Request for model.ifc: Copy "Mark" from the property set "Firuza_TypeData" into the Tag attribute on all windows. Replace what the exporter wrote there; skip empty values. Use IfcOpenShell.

First a look at what the model holds.

```python
import ifcopenshell
import ifcopenshell.util.element

model = ifcopenshell.open("model.ifc")
print(model.schema)
windows = model.by_type("IfcWindow")
print(len(windows), "windows")
for e in windows[:8]:
    source = ifcopenshell.util.element.get_pset(e, "Firuza_TypeData", "Mark")
    target = e.Tag
    print(e.id(), repr(source), repr(target), sep=" | ")
```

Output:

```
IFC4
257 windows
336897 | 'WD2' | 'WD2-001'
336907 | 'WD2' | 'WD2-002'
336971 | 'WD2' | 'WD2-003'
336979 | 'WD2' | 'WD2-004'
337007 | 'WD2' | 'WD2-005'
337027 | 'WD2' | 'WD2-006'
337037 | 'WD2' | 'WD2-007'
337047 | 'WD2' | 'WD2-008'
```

```python
import ifcopenshell
import ifcopenshell.util.element

model = ifcopenshell.open("model.ifc")

count = 0
for e in model.by_type("IfcWindow"):
    value = ifcopenshell.util.element.get_pset(e, "Firuza_TypeData", "Mark")
    current = e.Tag
    if not value or not value.strip() or current == value:
        continue
    e.Tag = value
    count += 1

print(count, "windows updated")

model.write("model_rev.ifc")
```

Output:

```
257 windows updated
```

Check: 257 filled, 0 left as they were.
